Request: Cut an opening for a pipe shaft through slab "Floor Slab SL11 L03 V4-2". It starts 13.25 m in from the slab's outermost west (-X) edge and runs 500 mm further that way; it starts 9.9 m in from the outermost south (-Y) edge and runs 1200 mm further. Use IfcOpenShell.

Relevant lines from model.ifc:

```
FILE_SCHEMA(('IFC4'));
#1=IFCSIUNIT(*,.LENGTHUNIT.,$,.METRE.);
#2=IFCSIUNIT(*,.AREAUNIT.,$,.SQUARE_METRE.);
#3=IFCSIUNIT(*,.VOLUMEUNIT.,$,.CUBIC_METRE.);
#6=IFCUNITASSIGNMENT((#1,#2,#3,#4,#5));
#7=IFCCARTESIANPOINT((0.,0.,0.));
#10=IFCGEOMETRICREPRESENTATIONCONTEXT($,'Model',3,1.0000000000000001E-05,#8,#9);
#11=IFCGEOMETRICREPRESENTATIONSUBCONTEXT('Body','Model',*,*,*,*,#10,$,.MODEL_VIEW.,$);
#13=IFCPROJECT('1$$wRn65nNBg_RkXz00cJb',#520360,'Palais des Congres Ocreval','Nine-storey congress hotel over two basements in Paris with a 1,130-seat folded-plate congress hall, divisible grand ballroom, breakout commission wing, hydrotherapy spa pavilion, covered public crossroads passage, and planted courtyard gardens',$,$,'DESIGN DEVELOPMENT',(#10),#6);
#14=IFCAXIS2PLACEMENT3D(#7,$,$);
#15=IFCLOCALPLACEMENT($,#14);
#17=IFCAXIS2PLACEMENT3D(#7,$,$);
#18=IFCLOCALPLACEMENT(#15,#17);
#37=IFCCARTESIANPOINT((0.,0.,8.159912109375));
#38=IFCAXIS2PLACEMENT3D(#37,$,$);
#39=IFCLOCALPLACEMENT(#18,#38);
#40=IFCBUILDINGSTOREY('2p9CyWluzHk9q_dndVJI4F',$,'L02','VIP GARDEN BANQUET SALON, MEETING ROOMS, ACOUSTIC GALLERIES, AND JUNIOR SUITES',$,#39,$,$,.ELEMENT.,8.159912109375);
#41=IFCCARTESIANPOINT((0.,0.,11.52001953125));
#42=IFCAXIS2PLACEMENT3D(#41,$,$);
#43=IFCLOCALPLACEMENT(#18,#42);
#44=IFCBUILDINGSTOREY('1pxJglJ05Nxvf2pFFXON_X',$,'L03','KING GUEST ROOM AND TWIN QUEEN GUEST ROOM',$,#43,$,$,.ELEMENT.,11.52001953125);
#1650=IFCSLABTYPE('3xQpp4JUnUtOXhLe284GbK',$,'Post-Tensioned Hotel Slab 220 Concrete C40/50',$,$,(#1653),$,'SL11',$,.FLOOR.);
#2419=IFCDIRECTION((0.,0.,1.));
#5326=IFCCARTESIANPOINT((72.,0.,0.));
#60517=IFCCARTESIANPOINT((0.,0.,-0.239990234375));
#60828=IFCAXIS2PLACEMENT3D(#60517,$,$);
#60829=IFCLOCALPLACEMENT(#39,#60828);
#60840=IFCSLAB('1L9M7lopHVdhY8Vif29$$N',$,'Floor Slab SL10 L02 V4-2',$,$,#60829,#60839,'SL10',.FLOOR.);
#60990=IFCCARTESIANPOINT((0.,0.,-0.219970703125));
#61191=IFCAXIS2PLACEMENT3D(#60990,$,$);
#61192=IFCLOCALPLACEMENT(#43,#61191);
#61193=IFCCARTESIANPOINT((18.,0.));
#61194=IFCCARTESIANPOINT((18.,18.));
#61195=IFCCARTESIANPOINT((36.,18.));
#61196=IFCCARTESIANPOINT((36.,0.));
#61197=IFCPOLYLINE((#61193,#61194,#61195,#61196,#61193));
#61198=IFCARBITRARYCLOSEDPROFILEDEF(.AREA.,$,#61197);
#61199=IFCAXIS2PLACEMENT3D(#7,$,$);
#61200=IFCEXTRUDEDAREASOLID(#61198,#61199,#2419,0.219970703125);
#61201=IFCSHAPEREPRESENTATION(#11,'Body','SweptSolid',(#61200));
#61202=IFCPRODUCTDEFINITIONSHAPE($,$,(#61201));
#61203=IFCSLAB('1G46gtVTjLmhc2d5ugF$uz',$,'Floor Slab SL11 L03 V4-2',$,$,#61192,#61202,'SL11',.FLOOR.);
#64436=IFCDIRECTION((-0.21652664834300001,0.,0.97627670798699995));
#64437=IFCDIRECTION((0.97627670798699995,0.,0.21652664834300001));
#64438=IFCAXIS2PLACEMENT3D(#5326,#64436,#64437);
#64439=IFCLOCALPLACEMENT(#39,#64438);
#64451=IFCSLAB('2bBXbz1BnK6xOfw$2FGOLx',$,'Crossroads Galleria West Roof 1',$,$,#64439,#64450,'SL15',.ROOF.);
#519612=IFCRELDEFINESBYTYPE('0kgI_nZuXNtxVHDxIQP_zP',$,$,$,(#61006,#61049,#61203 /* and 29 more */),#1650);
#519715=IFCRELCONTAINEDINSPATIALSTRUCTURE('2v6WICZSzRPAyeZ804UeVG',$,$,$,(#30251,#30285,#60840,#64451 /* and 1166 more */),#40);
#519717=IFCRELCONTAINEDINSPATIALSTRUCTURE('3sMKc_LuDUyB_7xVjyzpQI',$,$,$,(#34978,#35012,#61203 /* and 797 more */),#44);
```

```python
import numpy as np
import ifcopenshell
import ifcopenshell.api.feature
import ifcopenshell.api.geometry
import ifcopenshell.api.root
import ifcopenshell.geom
import ifcopenshell.util.placement
import ifcopenshell.util.representation
import ifcopenshell.util.shape
import ifcopenshell.util.unit

model = ifcopenshell.open("model.ifc")
unit_scale = ifcopenshell.util.unit.calculate_unit_scale(model)
settings = ifcopenshell.geom.settings()


def volume(element):
    """Net volume in cubic metres, openings subtracted."""
    shape = ifcopenshell.geom.create_shape(settings, element)
    return ifcopenshell.util.shape.get_volume(shape.geometry)


slab = model.by_guid("1G46gtVTjLmhc2d5ugF$uz")
before = volume(slab)

# Extent in the slab's own axes, in metres. The edges named are its -X and -Y sides.
slab_shape = ifcopenshell.geom.create_shape(settings, slab)
vertices = ifcopenshell.util.shape.get_vertices(slab_shape.geometry)
x_min, y_min, bottom = vertices.min(axis=0)
top = vertices[:, 2].max()

opening = ifcopenshell.api.root.create_entity(model, ifc_class="IfcOpeningElement", name="Pipe shaft opening", predefined_type="OPENING")
context = ifcopenshell.util.representation.get_context(model, "Model", "Body", "MODEL_VIEW")
width, depth = 0.5, 1.2
outline = [(0.0, 0.0), (width, 0.0), (width, depth), (0.0, depth), (0.0, 0.0)]
# Overshoot both faces by 50 mm so the cut is clean.
shape = ifcopenshell.api.geometry.add_slab_representation(
    model, context=context, depth=top - bottom + 0.1, polyline=outline
)
ifcopenshell.api.geometry.assign_representation(model, product=opening, representation=shape)

matrix = ifcopenshell.util.placement.get_local_placement(slab.ObjectPlacement)
matrix[:, 3] = matrix @ np.append(np.array([x_min + 13.25, y_min + 9.9, bottom - 0.05]) / unit_scale, 1.0)
ifcopenshell.api.geometry.edit_object_placement(model, product=opening, matrix=matrix, is_si=False)
ifcopenshell.api.feature.add_feature(model, feature=opening, element=slab)

after = volume(slab)

print(f"slab volume {before:.3f} -> {after:.3f} m3")

model.write("model-out.ifc")
```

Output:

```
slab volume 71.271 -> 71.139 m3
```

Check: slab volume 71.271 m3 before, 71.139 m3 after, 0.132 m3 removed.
